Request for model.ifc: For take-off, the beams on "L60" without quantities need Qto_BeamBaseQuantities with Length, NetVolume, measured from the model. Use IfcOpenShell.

First a look at what the model holds.

```python
import ifcopenshell
import ifcopenshell.util.element
import ifcopenshell.util.unit

model = ifcopenshell.open("model.ifc")
print(model.schema)
for unit_type in ("LENGTHUNIT", "AREAUNIT", "VOLUMEUNIT"):
    print(unit_type, ifcopenshell.util.unit.calculate_unit_scale(model, unit_type))
storey = next(s for s in model.by_type("IfcBuildingStorey") if s.Name == "L60")
beams = [e for e in ifcopenshell.util.element.get_decomposition(storey) if e.is_a("IfcBeam")]
for e in sorted(beams, key=lambda e: e.id()):
    print(e.id(), e.is_a(), e.Name, list(ifcopenshell.util.element.get_psets(e, qtos_only=True)), sep=" | ")
```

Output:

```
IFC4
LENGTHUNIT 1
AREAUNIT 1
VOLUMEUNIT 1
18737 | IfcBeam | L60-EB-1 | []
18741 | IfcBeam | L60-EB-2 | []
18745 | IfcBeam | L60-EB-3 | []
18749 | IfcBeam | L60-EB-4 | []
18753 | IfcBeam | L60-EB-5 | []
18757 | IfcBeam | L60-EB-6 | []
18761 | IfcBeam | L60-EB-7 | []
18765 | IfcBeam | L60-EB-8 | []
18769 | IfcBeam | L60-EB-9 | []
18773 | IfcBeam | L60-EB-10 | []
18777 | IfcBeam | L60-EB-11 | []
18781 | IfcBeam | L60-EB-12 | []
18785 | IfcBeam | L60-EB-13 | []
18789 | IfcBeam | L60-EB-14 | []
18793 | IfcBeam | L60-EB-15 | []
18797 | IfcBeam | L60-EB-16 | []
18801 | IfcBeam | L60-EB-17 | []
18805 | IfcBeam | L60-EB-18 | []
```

```python
import ifcopenshell
import ifcopenshell.api.pset
import ifcopenshell.geom
import ifcopenshell.util.element
import ifcopenshell.util.shape
import ifcopenshell.util.unit

model = ifcopenshell.open("model.ifc")
unit_scale = ifcopenshell.util.unit.calculate_unit_scale(model)
volume_scale = ifcopenshell.util.unit.calculate_unit_scale(model, "VOLUMEUNIT")
settings = ifcopenshell.geom.settings()

storey = next(s for s in model.by_type("IfcBuildingStorey") if s.Name == "L60")
beams = [e for e in ifcopenshell.util.element.get_decomposition(storey) if e.is_a("IfcBeam")]

for e in sorted(beams, key=lambda e: e.id()):
    if ifcopenshell.util.element.get_psets(e, qtos_only=True, should_inherit=False):
        continue
    # Geometry comes back in metres, in the element's own axes.
    shape = ifcopenshell.geom.create_shape(settings, e)
    values = {
        "Length": ifcopenshell.util.shape.get_max_xyz(shape.geometry) / unit_scale,
        "NetVolume": ifcopenshell.util.shape.get_volume(shape.geometry) / volume_scale,
    }
    qto = ifcopenshell.api.pset.add_qto(model, product=e, name="Qto_BeamBaseQuantities")
    ifcopenshell.api.pset.edit_qto(model, qto=qto, properties=values)
    print(e.id(), {k: round(v, 3) for k, v in values.items()})

model.write("model_v2.ifc")
```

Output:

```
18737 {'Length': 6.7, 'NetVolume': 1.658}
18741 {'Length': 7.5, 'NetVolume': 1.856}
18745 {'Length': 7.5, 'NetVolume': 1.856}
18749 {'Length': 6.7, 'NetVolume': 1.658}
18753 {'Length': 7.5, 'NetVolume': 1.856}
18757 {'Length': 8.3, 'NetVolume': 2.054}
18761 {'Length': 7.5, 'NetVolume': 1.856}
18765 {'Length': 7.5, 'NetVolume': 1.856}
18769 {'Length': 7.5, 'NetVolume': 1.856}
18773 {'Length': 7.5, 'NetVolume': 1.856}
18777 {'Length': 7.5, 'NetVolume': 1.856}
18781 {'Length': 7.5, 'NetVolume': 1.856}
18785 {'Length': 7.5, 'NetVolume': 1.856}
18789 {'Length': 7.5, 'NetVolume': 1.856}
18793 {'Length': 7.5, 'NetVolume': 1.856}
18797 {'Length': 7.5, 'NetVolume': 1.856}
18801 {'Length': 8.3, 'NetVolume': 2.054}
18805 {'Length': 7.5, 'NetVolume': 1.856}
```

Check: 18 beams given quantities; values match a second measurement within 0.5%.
